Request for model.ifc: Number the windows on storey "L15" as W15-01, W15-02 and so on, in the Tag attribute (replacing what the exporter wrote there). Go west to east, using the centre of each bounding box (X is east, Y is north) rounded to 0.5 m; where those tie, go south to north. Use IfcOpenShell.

First a look at what the model holds.

```python
import ifcopenshell
import ifcopenshell.util.element
import ifcopenshell.util.placement

model = ifcopenshell.open("model.ifc")
print(model.schema)
storey = next(s for s in model.by_type("IfcBuildingStorey") if s.Name == "L15")
windows = [e for e in ifcopenshell.util.element.get_decomposition(storey) if e.is_a("IfcWindow")]
for e in sorted(windows, key=lambda e: e.id()):
    origin = ifcopenshell.util.placement.get_local_placement(e.ObjectPlacement)[:3, 3]
    print(e.id(), e.Tag, e.Name, origin.round(2) + 0.0, sep=" | ")
```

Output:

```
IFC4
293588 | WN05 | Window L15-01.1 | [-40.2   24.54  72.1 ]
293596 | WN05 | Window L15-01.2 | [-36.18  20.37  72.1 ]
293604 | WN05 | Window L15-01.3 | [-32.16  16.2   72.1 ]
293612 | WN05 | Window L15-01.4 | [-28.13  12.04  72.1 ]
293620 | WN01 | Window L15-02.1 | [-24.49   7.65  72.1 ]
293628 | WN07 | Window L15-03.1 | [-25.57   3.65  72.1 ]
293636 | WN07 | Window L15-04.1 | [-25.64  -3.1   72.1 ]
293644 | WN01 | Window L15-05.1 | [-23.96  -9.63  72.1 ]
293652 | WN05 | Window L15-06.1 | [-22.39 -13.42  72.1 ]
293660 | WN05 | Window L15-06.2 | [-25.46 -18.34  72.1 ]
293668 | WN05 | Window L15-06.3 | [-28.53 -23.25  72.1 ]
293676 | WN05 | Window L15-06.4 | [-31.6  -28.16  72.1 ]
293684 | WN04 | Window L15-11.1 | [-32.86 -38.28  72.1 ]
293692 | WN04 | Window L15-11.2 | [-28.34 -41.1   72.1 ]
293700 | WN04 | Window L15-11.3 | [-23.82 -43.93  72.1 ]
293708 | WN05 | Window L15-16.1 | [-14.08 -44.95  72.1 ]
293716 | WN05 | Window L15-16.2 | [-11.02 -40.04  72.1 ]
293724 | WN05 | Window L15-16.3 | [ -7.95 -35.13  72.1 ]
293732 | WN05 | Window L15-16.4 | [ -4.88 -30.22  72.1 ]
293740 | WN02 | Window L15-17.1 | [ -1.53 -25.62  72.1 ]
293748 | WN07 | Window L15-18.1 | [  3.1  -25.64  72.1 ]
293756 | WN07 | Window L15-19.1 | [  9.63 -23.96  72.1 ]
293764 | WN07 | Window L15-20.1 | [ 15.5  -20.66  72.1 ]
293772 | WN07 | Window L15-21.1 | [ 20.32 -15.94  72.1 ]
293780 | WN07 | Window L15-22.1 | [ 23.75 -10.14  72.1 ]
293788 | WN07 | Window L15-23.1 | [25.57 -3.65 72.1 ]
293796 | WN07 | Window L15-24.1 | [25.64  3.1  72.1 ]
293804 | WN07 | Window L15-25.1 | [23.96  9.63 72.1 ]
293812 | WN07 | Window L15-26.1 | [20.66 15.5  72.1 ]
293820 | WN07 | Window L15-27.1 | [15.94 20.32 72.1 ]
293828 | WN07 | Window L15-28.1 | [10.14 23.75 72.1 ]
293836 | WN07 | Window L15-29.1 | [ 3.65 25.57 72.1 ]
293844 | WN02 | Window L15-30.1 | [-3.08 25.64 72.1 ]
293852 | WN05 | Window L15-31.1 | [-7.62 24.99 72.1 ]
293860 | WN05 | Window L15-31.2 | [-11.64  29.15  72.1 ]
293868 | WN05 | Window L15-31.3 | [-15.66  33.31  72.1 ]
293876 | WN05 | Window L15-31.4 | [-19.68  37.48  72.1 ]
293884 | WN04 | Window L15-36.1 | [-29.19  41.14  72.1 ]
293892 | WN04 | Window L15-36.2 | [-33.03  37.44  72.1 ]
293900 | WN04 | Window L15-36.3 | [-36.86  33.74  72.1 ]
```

```python
import ifcopenshell
import ifcopenshell.geom
import ifcopenshell.util.element
import ifcopenshell.util.shape

model = ifcopenshell.open("model.ifc")
settings = ifcopenshell.geom.settings()
settings.set("use-world-coords", True)


def centre(element):
    shape = ifcopenshell.geom.create_shape(settings, element)
    return ifcopenshell.util.shape.get_bbox_centroid(shape.geometry)


storey = next(s for s in model.by_type("IfcBuildingStorey") if s.Name == "L15")
windows = [e for e in ifcopenshell.util.element.get_decomposition(storey) if e.is_a("IfcWindow")]

# Insertion points can sit at a corner or the storey origin, so sort by the geometry (in metres).
centres = {e: centre(e) for e in windows}
windows.sort(key=lambda e: (round(centres[e][0] / 0.5), centres[e][1]))

for i, e in enumerate(windows, start=1):
    number = f"W15-{i:02d}"
    e.Tag = number
    print(e.id(), number)

model.write("model_edited.ifc")
```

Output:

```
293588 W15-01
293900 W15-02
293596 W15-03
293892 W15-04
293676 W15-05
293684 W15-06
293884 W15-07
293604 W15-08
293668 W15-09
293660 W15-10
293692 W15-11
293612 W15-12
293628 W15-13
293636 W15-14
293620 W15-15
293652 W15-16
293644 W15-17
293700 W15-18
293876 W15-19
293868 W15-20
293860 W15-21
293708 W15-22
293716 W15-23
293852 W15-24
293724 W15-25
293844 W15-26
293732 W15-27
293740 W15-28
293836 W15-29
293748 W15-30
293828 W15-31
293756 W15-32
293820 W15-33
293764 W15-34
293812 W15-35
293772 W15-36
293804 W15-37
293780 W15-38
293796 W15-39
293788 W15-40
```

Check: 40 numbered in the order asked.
